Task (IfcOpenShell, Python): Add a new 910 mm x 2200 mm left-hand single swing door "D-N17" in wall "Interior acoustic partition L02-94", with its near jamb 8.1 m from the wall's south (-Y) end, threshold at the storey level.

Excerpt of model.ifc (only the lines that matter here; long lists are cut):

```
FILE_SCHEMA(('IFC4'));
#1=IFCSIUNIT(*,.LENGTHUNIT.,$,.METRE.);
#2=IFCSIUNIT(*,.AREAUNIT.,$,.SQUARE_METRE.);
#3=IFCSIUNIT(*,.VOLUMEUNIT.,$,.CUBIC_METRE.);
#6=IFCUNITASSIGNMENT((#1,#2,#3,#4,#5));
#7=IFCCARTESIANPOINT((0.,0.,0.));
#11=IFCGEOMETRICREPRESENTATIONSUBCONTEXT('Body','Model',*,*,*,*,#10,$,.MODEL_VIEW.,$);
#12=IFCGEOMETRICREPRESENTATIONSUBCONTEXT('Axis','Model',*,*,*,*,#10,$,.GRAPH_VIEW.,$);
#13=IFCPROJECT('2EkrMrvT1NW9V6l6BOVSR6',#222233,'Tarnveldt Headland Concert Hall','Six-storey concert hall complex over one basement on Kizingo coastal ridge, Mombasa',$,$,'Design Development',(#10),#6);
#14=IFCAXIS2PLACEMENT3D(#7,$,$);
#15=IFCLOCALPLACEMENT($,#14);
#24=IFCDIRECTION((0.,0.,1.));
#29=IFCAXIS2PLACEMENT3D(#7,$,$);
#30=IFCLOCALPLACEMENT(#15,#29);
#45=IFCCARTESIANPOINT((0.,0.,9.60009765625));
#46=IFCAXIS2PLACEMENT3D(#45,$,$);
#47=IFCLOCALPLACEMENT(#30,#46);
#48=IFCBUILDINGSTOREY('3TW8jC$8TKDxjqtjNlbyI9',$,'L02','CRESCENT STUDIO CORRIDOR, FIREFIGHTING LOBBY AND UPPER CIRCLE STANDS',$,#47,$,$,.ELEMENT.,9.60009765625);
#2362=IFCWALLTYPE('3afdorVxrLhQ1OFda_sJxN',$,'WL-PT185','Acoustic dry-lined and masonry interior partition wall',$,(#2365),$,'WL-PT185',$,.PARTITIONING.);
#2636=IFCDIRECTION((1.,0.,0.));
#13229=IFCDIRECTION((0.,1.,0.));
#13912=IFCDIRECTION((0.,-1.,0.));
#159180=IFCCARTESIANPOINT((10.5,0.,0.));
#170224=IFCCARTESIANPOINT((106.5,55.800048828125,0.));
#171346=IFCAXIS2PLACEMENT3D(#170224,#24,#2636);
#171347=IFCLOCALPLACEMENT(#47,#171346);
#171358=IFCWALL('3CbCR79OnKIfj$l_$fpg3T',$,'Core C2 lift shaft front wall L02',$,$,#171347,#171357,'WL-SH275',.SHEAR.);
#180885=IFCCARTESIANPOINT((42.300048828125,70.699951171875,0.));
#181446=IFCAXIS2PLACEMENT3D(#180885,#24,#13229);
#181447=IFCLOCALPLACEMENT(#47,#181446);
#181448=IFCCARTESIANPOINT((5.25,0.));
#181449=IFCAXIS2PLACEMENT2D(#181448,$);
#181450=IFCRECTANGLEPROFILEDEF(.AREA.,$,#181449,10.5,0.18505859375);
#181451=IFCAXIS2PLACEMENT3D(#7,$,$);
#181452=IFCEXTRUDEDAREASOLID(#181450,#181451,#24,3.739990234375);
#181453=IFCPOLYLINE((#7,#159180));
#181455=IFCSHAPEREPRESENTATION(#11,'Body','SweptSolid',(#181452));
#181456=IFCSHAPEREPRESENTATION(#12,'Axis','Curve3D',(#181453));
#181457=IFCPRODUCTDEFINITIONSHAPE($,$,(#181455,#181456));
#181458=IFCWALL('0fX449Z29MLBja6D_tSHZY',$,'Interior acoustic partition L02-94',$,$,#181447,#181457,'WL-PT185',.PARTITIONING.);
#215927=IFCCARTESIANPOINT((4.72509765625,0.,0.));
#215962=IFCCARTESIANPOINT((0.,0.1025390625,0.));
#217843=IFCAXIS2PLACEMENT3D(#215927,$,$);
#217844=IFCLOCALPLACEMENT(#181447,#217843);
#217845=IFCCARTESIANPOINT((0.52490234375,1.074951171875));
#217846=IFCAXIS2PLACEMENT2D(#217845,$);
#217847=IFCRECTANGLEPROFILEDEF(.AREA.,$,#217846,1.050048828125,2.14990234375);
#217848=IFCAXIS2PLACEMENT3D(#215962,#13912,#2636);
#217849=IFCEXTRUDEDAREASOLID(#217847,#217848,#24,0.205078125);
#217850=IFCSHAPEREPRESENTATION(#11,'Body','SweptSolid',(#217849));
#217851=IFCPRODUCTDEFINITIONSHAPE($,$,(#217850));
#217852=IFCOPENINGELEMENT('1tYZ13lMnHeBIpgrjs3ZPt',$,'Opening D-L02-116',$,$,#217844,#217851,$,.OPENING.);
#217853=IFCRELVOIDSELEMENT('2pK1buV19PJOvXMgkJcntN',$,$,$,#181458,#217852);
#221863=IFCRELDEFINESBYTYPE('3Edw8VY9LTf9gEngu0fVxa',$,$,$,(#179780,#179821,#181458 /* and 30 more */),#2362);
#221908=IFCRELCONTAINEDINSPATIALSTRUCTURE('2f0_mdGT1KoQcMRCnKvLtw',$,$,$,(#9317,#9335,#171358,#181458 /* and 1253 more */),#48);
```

```python
import numpy as np
import ifcopenshell
import ifcopenshell.api.feature
import ifcopenshell.api.geometry
import ifcopenshell.api.root
import ifcopenshell.api.spatial
import ifcopenshell.geom
import ifcopenshell.util.element
import ifcopenshell.util.placement
import ifcopenshell.util.representation
import ifcopenshell.util.shape
import ifcopenshell.util.unit

model = ifcopenshell.open("model.ifc")
unit_scale = ifcopenshell.util.unit.calculate_unit_scale(model)
settings = ifcopenshell.geom.settings()


def volume(element):
    """Net volume in cubic metres, openings subtracted."""
    shape = ifcopenshell.geom.create_shape(settings, element)
    return ifcopenshell.util.shape.get_volume(shape.geometry)


wall = model.by_guid("0fX449Z29MLBja6D_tSHZY")
storey = ifcopenshell.util.element.get_container(wall, ifc_class="IfcBuildingStorey")
context = ifcopenshell.util.representation.get_context(model, "Model", "Body", "MODEL_VIEW")
before = volume(wall)

width, height, from_end, sill = 0.91, 2.2, 8.1, 0.0  # metres

# The wall runs along its own X axis, and the end named is its -X end.
wall_shape = ifcopenshell.geom.create_shape(settings, wall)
x, y, z = ifcopenshell.util.shape.get_vertices(wall_shape.geometry).T
start = x.min() + from_end
face, thickness = float(y.min()), float(y.max() - y.min())
wall_matrix = ifcopenshell.util.placement.get_local_placement(wall.ObjectPlacement)
level = ifcopenshell.util.placement.get_local_placement(storey.ObjectPlacement)[2, 3]


def in_wall(x, y):
    """Placement at x, y metres in the wall's axes, at sill height."""
    matrix = wall_matrix.copy()
    matrix[:, 3] = wall_matrix @ np.array([x / unit_scale, y / unit_scale, 0.0, 1.0])
    matrix[2, 3] = level + sill / unit_scale
    return matrix


# Opening: a box that overshoots both wall faces by 50 mm.
opening = ifcopenshell.api.root.create_entity(model, ifc_class="IfcOpeningElement", predefined_type="OPENING")
box = ifcopenshell.api.geometry.add_wall_representation(
    model, context=context, length=width, height=height, thickness=thickness + 0.1
)
ifcopenshell.api.geometry.assign_representation(model, product=opening, representation=box)
ifcopenshell.api.geometry.edit_object_placement(model, product=opening, matrix=in_wall(start, face - 0.05), is_si=False)
ifcopenshell.api.feature.add_feature(model, feature=opening, element=wall)

door = ifcopenshell.api.root.create_entity(model, ifc_class="IfcDoor", name="D-N17", predefined_type="DOOR")
door.OverallWidth, door.OverallHeight = width / unit_scale, height / unit_scale
door.OperationType = "SINGLE_SWING_LEFT"
body = ifcopenshell.api.geometry.add_door_representation(
    model,
    context=context,
    overall_width=door.OverallWidth,
    overall_height=door.OverallHeight,
    operation_type="SINGLE_SWING_LEFT",
    lining_properties={"LiningDepth": thickness / unit_scale, "ThresholdDepth": thickness / unit_scale},
)
ifcopenshell.api.geometry.assign_representation(model, product=door, representation=body)
ifcopenshell.api.spatial.assign_container(model, products=[door], relating_structure=storey)
ifcopenshell.api.feature.add_filling(model, opening=opening, element=door)

# The lining spans the wall, so the door starts at the wall face.
ifcopenshell.api.geometry.edit_object_placement(model, product=door, matrix=in_wall(start, face), is_si=False)

after = volume(wall)

print(f"wall volume {before:.3f} -> {after:.3f} m3")

model.write("model_updated.ifc")
```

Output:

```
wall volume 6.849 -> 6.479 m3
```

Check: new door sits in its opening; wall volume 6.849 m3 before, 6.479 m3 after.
